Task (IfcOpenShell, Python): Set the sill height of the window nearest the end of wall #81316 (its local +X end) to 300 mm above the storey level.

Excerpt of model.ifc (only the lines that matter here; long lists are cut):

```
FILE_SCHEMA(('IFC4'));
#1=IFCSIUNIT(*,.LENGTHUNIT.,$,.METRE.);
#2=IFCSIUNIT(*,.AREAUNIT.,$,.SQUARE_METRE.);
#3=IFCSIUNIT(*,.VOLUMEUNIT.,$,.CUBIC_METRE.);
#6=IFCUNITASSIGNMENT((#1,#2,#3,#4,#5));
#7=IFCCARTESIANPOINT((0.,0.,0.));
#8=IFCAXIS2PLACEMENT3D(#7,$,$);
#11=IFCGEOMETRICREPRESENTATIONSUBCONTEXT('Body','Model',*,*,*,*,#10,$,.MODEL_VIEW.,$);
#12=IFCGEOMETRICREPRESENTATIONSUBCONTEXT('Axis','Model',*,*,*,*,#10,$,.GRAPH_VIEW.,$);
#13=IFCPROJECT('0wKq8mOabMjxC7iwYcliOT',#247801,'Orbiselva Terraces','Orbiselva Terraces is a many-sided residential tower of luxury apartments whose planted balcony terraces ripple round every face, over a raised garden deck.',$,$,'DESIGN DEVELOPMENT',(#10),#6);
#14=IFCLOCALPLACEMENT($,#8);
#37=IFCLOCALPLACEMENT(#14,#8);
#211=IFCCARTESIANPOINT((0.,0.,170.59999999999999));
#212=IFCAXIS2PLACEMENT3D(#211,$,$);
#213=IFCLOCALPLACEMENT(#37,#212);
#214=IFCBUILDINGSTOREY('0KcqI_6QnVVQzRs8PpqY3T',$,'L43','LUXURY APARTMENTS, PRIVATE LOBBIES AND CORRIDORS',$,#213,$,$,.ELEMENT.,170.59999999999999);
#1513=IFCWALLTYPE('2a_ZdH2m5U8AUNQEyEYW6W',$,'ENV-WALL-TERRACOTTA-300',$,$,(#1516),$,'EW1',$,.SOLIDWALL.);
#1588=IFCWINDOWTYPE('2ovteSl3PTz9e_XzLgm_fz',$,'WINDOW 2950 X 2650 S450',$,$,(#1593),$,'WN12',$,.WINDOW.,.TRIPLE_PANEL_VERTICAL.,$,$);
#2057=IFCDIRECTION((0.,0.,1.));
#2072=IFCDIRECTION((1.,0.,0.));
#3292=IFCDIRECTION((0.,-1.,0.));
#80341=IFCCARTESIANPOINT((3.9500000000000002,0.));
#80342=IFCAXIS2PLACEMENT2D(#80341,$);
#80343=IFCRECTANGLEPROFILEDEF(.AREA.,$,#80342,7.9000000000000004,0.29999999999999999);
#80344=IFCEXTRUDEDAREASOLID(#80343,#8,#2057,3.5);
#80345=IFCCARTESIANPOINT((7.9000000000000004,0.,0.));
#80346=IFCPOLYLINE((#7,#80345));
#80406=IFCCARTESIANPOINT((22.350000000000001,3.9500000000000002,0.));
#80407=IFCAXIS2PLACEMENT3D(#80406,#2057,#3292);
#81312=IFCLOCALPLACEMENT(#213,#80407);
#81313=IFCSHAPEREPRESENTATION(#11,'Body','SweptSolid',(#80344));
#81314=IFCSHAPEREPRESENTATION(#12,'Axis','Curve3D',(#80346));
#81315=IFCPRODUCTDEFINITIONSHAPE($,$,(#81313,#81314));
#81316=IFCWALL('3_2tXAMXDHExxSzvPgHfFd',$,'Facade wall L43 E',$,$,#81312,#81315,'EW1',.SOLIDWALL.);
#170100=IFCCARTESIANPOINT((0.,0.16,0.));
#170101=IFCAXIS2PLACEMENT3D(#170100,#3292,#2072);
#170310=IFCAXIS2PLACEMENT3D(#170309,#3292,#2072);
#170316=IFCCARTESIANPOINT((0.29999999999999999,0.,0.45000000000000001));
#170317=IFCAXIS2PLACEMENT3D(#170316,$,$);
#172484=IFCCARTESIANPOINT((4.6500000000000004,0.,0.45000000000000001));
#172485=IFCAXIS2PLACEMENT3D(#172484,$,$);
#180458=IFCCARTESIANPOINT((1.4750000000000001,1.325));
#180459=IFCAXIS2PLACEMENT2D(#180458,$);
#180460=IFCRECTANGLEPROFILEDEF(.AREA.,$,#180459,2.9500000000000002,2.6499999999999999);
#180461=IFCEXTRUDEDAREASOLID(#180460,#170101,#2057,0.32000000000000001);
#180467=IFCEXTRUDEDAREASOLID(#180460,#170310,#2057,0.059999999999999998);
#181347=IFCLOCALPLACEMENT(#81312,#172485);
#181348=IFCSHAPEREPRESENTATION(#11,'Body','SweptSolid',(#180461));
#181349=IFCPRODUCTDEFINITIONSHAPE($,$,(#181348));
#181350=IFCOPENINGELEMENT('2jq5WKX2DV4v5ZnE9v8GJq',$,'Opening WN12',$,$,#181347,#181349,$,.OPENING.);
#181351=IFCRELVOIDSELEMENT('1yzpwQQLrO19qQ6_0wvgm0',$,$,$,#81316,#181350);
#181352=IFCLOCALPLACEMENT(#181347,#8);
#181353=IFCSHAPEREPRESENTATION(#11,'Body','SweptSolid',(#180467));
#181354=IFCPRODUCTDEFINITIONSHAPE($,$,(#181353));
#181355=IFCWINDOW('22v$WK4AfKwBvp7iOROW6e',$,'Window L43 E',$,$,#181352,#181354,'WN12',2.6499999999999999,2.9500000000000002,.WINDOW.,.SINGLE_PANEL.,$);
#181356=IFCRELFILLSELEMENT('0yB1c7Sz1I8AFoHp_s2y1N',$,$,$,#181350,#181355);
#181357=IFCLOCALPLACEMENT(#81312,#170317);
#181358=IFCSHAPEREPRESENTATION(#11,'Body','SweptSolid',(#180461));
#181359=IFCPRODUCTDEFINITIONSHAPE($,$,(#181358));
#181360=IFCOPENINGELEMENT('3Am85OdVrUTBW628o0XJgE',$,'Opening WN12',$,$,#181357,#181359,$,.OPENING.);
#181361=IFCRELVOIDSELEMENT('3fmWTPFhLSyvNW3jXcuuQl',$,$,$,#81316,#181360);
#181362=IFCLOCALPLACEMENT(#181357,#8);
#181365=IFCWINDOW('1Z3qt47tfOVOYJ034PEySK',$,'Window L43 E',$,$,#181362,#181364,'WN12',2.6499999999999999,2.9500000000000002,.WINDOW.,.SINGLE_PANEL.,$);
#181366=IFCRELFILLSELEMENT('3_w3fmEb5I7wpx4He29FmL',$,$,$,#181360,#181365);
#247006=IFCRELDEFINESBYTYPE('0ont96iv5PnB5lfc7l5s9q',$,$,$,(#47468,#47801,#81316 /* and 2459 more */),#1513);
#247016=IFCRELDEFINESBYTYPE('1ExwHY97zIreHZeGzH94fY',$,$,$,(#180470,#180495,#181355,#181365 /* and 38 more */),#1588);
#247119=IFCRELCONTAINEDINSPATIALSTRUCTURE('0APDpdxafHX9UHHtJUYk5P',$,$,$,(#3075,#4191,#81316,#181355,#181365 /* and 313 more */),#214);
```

```python
import numpy as np
import ifcopenshell
import ifcopenshell.api.geometry
import ifcopenshell.geom
import ifcopenshell.util.element
import ifcopenshell.util.placement
import ifcopenshell.util.shape
import ifcopenshell.util.unit

model = ifcopenshell.open("model.ifc")
unit_scale = ifcopenshell.util.unit.calculate_unit_scale(model)

window = model.by_guid("22v$WK4AfKwBvp7iOROW6e")
opening = window.FillsVoids[0].RelatingOpeningElement
storey = ifcopenshell.util.element.get_container(window, ifc_class="IfcBuildingStorey")
level = ifcopenshell.util.placement.get_local_placement(storey.ObjectPlacement)[2, 3]

# The opening's origin need not be at the sill, so measure its lowest point.
shape = ifcopenshell.geom.create_shape(ifcopenshell.geom.settings(), opening)
bottom = ifcopenshell.util.shape.get_shape_bottom_elevation(shape, shape.geometry) / unit_scale
dz = level + 0.3 / unit_scale - bottom

shift = np.array([0.0, 0.0, dz])
# The window is placed relative to its opening, so it follows when the opening moves.
matrix = ifcopenshell.util.placement.get_local_placement(opening.ObjectPlacement)
matrix[:3, 3] += shift
ifcopenshell.api.geometry.edit_object_placement(
    model, product=opening, matrix=matrix, is_si=False, should_transform_children=True
)

print(f"moved by {dz * unit_scale:+.3f} m")

model.write("model_v2.ifc")
```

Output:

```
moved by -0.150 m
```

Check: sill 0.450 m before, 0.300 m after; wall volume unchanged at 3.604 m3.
